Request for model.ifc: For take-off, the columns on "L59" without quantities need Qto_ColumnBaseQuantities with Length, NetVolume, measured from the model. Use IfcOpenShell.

First a look at what the model holds.

```python
import ifcopenshell
import ifcopenshell.util.element
import ifcopenshell.util.unit

model = ifcopenshell.open("model.ifc")
print(model.schema)
for unit_type in ("LENGTHUNIT", "AREAUNIT", "VOLUMEUNIT"):
    print(unit_type, ifcopenshell.util.unit.calculate_unit_scale(model, unit_type))
storey = next(s for s in model.by_type("IfcBuildingStorey") if s.Name == "L59")
columns = [e for e in ifcopenshell.util.element.get_decomposition(storey) if e.is_a("IfcColumn")]
for e in sorted(columns, key=lambda e: e.id()):
    print(e.id(), e.is_a(), e.Name, list(ifcopenshell.util.element.get_psets(e, qtos_only=True)), sep=" | ")
```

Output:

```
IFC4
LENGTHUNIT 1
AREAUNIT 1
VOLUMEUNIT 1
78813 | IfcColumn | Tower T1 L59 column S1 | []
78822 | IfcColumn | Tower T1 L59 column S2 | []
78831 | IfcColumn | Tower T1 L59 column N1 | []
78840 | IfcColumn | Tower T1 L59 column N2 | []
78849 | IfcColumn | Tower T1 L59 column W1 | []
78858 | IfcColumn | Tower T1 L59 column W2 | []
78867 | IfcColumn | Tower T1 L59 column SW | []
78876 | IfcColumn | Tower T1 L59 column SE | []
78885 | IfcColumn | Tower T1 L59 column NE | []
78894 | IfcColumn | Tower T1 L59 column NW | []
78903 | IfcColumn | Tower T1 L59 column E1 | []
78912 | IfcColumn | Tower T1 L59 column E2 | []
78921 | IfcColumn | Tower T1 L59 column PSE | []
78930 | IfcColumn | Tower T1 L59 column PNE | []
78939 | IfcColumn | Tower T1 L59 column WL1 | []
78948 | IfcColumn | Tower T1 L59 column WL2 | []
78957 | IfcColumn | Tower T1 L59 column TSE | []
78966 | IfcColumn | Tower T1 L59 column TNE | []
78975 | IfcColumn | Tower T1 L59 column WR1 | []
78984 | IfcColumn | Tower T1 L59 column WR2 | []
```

```python
import ifcopenshell
import ifcopenshell.api.pset
import ifcopenshell.geom
import ifcopenshell.util.element
import ifcopenshell.util.shape
import ifcopenshell.util.unit

model = ifcopenshell.open("model.ifc")
unit_scale = ifcopenshell.util.unit.calculate_unit_scale(model)
volume_scale = ifcopenshell.util.unit.calculate_unit_scale(model, "VOLUMEUNIT")
settings = ifcopenshell.geom.settings()

storey = next(s for s in model.by_type("IfcBuildingStorey") if s.Name == "L59")
columns = [e for e in ifcopenshell.util.element.get_decomposition(storey) if e.is_a("IfcColumn")]

for e in sorted(columns, key=lambda e: e.id()):
    if ifcopenshell.util.element.get_psets(e, qtos_only=True, should_inherit=False):
        continue
    # Geometry comes back in metres, in the element's own axes.
    shape = ifcopenshell.geom.create_shape(settings, e)
    values = {
        "Length": ifcopenshell.util.shape.get_z(shape.geometry) / unit_scale,
        "NetVolume": ifcopenshell.util.shape.get_volume(shape.geometry) / volume_scale,
    }
    qto = ifcopenshell.api.pset.add_qto(model, product=e, name="Qto_ColumnBaseQuantities")
    ifcopenshell.api.pset.edit_qto(model, qto=qto, properties=values)
    print(e.id(), {k: round(v, 3) for k, v in values.items()})

model.write("model_rev.ifc")
```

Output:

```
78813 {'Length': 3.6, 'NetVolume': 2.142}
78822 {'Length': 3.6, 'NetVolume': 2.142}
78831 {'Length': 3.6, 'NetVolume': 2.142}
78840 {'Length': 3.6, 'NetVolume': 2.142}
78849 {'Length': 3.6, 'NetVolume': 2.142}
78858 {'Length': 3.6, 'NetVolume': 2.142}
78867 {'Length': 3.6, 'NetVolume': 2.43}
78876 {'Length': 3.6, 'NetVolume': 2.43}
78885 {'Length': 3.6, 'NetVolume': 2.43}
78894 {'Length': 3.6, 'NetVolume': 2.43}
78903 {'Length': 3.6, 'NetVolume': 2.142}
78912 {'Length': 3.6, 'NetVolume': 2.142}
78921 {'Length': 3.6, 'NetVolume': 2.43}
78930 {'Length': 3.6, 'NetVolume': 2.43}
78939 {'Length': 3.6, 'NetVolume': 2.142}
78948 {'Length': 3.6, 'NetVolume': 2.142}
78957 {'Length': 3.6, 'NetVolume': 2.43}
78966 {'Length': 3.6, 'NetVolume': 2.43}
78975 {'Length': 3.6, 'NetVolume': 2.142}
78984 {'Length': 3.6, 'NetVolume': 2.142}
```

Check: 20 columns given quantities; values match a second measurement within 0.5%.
